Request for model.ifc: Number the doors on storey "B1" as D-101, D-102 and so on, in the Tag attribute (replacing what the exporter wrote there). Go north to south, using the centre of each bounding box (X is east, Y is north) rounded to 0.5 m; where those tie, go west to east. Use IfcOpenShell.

First a look at what the model holds.

```python
import ifcopenshell
import ifcopenshell.util.element
import ifcopenshell.util.placement

model = ifcopenshell.open("model.ifc")
print(model.schema)
storey = next(s for s in model.by_type("IfcBuildingStorey") if s.Name == "B1")
doors = [e for e in ifcopenshell.util.element.get_decomposition(storey) if e.is_a("IfcDoor")]
for e in sorted(doors, key=lambda e: e.id()):
    origin = ifcopenshell.util.placement.get_local_placement(e.ObjectPlacement)[:3, 3]
    print(e.id(), e.Tag, e.Name, origin.round(2) + 0.0, sep=" | ")
```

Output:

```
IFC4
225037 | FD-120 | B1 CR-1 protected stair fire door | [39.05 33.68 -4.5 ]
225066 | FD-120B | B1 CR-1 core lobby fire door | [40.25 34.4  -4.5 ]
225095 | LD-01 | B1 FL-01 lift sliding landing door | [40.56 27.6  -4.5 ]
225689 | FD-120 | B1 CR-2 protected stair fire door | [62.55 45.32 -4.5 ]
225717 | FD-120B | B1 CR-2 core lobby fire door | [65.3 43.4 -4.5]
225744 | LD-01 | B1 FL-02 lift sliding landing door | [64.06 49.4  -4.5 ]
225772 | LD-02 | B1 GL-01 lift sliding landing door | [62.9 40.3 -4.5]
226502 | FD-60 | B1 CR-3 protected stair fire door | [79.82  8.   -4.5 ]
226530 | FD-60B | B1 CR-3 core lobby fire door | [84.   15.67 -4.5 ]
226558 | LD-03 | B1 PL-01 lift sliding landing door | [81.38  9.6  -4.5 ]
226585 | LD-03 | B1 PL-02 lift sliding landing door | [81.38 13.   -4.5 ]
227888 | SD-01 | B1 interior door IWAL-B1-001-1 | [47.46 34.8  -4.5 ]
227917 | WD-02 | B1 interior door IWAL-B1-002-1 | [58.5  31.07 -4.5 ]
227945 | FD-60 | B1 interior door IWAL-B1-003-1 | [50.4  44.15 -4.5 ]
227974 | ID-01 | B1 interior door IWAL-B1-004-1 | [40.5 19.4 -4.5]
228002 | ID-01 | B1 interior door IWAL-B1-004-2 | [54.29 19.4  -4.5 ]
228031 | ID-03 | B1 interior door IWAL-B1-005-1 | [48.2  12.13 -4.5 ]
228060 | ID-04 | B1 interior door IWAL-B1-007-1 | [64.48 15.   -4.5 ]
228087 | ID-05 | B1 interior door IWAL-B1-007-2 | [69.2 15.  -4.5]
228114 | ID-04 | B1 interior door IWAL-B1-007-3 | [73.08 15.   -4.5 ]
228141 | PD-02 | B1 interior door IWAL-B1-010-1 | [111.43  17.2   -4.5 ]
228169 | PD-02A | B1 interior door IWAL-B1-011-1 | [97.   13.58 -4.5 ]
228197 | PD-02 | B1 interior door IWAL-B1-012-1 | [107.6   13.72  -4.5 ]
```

```python
import ifcopenshell
import ifcopenshell.geom
import ifcopenshell.util.element
import ifcopenshell.util.shape

model = ifcopenshell.open("model.ifc")
settings = ifcopenshell.geom.settings()
settings.set("use-world-coords", True)


def centre(element):
    shape = ifcopenshell.geom.create_shape(settings, element)
    return ifcopenshell.util.shape.get_bbox_centroid(shape.geometry)


storey = next(s for s in model.by_type("IfcBuildingStorey") if s.Name == "B1")
doors = [e for e in ifcopenshell.util.element.get_decomposition(storey) if e.is_a("IfcDoor")]

# Insertion points can sit at a corner or the storey origin, so sort by the geometry (in metres).
centres = {e: centre(e) for e in doors}
doors.sort(key=lambda e: (-round(centres[e][1] / 0.5), centres[e][0]))

for i, e in enumerate(doors, start=1):
    number = f"D-1{i:02d}"
    e.Tag = number
    print(e.id(), number)

model.write("model_edited.ifc")
```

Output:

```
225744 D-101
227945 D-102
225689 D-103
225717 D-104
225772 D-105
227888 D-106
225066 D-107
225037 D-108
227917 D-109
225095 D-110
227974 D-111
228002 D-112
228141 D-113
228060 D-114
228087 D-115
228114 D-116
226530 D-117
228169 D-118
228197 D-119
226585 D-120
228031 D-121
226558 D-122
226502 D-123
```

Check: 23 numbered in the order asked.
